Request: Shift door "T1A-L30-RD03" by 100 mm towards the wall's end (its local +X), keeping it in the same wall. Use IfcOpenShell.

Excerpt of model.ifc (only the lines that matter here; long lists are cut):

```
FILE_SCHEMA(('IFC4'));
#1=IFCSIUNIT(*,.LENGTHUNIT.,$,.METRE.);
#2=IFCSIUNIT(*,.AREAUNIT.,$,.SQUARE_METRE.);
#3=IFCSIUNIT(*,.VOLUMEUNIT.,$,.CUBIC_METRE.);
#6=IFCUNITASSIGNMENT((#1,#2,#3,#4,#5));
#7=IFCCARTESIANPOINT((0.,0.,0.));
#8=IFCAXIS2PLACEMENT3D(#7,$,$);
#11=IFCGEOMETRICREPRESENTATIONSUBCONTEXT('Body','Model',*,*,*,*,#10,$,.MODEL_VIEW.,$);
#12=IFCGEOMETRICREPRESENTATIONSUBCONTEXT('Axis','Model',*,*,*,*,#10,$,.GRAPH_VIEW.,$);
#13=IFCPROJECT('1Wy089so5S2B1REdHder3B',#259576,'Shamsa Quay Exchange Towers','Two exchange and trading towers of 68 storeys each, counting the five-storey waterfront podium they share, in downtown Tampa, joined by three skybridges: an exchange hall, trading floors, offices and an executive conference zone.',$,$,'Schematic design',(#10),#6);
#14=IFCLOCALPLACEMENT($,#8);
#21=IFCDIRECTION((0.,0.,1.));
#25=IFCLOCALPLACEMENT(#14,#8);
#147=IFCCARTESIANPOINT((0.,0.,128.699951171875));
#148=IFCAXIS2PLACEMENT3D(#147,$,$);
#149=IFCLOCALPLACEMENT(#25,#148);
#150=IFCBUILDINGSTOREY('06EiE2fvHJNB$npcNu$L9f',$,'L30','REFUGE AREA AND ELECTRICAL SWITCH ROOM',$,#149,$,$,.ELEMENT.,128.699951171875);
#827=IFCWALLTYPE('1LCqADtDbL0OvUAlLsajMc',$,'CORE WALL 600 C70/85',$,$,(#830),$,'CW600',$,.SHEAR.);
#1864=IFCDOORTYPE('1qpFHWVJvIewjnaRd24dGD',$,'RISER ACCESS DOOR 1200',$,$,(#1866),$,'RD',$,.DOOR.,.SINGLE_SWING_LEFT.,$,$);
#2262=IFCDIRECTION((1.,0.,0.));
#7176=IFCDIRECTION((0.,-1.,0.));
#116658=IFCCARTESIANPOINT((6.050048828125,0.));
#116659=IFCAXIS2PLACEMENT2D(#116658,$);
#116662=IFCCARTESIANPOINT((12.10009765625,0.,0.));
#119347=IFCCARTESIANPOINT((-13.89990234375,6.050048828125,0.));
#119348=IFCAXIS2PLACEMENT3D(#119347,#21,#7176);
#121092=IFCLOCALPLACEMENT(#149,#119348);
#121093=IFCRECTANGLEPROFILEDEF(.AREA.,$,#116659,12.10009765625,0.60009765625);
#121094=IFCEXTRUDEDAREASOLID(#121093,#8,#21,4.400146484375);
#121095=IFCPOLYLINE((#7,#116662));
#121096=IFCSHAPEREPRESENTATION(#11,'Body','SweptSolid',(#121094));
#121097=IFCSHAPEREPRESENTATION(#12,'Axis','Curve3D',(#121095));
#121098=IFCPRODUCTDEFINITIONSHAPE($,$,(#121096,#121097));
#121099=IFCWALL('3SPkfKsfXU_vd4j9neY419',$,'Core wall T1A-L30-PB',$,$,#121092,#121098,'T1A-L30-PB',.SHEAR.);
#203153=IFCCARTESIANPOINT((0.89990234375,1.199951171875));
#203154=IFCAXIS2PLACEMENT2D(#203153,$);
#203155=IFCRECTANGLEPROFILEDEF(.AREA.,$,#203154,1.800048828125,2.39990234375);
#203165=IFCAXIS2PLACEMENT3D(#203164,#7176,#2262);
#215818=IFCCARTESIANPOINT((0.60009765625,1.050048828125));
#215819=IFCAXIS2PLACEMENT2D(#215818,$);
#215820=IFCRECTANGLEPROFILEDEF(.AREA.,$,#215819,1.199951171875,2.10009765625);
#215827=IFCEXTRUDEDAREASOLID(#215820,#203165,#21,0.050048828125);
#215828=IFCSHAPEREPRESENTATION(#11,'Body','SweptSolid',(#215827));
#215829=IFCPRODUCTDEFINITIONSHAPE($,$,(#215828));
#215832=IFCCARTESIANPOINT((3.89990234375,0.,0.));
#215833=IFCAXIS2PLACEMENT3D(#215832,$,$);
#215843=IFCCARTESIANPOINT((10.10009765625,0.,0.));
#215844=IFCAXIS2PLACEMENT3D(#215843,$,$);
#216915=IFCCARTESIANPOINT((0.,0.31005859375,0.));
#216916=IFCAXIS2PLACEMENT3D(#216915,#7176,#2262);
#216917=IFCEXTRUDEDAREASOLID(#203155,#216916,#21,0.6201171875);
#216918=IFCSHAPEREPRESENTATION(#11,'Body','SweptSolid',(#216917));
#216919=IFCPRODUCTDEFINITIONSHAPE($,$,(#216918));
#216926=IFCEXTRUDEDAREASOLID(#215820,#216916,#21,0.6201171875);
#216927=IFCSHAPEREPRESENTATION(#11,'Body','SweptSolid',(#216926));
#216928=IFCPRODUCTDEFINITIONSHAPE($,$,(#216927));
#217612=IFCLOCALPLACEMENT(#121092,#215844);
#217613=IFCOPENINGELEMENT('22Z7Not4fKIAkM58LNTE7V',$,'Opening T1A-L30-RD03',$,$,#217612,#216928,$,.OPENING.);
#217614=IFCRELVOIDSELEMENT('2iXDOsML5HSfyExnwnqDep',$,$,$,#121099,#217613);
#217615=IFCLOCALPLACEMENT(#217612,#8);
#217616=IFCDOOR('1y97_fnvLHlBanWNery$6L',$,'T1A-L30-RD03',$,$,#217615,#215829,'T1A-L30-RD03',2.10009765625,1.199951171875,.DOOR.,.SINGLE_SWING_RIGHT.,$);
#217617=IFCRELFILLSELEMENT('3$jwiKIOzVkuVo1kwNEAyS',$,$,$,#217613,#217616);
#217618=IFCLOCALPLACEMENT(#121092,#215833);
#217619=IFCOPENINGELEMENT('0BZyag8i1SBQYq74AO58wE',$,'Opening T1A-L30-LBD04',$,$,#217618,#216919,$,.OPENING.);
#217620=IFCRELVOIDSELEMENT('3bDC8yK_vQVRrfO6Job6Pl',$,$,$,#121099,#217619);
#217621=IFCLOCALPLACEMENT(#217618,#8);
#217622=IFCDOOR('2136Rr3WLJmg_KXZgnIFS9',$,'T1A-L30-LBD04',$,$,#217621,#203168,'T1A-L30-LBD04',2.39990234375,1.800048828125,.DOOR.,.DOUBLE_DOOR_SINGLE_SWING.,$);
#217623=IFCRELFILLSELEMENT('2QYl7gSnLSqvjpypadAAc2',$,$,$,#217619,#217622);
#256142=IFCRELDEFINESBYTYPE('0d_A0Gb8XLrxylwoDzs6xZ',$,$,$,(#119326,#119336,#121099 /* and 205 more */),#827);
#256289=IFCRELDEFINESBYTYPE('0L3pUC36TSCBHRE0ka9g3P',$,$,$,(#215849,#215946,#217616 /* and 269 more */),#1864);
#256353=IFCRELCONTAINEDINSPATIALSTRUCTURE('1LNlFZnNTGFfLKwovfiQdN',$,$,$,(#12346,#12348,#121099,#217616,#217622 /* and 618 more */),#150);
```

```python
import ifcopenshell
import ifcopenshell.api.geometry
import ifcopenshell.util.placement

model = ifcopenshell.open("model.ifc")

door = model.by_guid("1y97_fnvLHlBanWNery$6L")
opening = door.FillsVoids[0].RelatingOpeningElement
wall = opening.VoidsElements[0].RelatingBuildingElement

wall_matrix = ifcopenshell.util.placement.get_local_placement(wall.ObjectPlacement)
shift = wall_matrix[:3, 0] * 0.1
before = ifcopenshell.util.placement.get_local_placement(door.ObjectPlacement)[:3, 3].copy()

# The door is placed relative to its opening, so it follows when the opening moves.
matrix = ifcopenshell.util.placement.get_local_placement(opening.ObjectPlacement)
matrix[:3, 3] += shift
ifcopenshell.api.geometry.edit_object_placement(
    model, product=opening, matrix=matrix, is_si=False, should_transform_children=True
)

after = ifcopenshell.util.placement.get_local_placement(door.ObjectPlacement)[:3, 3]
print("door moved by", (after - before).round(3) + 0.0)

model.write("model_updated.ifc")
```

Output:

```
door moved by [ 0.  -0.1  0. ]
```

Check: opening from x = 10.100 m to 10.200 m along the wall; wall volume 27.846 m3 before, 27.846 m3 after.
